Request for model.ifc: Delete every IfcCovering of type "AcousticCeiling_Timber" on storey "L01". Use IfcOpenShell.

First a look at what the model holds.

```python
import ifcopenshell
import ifcopenshell.util.element

model = ifcopenshell.open("model.ifc")
print(model.schema)
storey = next(s for s in model.by_type("IfcBuildingStorey") if s.Name == "L01")
coverings = [e for e in ifcopenshell.util.element.get_decomposition(storey) if e.is_a("IfcCovering")]
seen = {}
for e in coverings:
    element_type = ifcopenshell.util.element.get_type(e)
    name = element_type.Name if element_type not in (None, e) else None
    seen[name] = seen.get(name, 0) + 1
for name, count in sorted(seen.items(), key=str):
    print(count, "x", name)
```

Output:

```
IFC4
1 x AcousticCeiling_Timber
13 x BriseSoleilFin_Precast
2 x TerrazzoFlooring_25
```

```python
import ifcopenshell
import ifcopenshell.api.root
import ifcopenshell.util.element

model = ifcopenshell.open("model.ifc")

storey = next(s for s in model.by_type("IfcBuildingStorey") if s.Name == "L01")
coverings = [e for e in ifcopenshell.util.element.get_decomposition(storey) if e.is_a("IfcCovering")]
targets = [e for e in coverings if (t := ifcopenshell.util.element.get_type(e)) not in (None, e) and t.Name == "AcousticCeiling_Timber"]

for e in targets:
    ifcopenshell.api.root.remove_product(model, product=e)
print(len(targets), "removed")

model.write("model_v2.ifc")
```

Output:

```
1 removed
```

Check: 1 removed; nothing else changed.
